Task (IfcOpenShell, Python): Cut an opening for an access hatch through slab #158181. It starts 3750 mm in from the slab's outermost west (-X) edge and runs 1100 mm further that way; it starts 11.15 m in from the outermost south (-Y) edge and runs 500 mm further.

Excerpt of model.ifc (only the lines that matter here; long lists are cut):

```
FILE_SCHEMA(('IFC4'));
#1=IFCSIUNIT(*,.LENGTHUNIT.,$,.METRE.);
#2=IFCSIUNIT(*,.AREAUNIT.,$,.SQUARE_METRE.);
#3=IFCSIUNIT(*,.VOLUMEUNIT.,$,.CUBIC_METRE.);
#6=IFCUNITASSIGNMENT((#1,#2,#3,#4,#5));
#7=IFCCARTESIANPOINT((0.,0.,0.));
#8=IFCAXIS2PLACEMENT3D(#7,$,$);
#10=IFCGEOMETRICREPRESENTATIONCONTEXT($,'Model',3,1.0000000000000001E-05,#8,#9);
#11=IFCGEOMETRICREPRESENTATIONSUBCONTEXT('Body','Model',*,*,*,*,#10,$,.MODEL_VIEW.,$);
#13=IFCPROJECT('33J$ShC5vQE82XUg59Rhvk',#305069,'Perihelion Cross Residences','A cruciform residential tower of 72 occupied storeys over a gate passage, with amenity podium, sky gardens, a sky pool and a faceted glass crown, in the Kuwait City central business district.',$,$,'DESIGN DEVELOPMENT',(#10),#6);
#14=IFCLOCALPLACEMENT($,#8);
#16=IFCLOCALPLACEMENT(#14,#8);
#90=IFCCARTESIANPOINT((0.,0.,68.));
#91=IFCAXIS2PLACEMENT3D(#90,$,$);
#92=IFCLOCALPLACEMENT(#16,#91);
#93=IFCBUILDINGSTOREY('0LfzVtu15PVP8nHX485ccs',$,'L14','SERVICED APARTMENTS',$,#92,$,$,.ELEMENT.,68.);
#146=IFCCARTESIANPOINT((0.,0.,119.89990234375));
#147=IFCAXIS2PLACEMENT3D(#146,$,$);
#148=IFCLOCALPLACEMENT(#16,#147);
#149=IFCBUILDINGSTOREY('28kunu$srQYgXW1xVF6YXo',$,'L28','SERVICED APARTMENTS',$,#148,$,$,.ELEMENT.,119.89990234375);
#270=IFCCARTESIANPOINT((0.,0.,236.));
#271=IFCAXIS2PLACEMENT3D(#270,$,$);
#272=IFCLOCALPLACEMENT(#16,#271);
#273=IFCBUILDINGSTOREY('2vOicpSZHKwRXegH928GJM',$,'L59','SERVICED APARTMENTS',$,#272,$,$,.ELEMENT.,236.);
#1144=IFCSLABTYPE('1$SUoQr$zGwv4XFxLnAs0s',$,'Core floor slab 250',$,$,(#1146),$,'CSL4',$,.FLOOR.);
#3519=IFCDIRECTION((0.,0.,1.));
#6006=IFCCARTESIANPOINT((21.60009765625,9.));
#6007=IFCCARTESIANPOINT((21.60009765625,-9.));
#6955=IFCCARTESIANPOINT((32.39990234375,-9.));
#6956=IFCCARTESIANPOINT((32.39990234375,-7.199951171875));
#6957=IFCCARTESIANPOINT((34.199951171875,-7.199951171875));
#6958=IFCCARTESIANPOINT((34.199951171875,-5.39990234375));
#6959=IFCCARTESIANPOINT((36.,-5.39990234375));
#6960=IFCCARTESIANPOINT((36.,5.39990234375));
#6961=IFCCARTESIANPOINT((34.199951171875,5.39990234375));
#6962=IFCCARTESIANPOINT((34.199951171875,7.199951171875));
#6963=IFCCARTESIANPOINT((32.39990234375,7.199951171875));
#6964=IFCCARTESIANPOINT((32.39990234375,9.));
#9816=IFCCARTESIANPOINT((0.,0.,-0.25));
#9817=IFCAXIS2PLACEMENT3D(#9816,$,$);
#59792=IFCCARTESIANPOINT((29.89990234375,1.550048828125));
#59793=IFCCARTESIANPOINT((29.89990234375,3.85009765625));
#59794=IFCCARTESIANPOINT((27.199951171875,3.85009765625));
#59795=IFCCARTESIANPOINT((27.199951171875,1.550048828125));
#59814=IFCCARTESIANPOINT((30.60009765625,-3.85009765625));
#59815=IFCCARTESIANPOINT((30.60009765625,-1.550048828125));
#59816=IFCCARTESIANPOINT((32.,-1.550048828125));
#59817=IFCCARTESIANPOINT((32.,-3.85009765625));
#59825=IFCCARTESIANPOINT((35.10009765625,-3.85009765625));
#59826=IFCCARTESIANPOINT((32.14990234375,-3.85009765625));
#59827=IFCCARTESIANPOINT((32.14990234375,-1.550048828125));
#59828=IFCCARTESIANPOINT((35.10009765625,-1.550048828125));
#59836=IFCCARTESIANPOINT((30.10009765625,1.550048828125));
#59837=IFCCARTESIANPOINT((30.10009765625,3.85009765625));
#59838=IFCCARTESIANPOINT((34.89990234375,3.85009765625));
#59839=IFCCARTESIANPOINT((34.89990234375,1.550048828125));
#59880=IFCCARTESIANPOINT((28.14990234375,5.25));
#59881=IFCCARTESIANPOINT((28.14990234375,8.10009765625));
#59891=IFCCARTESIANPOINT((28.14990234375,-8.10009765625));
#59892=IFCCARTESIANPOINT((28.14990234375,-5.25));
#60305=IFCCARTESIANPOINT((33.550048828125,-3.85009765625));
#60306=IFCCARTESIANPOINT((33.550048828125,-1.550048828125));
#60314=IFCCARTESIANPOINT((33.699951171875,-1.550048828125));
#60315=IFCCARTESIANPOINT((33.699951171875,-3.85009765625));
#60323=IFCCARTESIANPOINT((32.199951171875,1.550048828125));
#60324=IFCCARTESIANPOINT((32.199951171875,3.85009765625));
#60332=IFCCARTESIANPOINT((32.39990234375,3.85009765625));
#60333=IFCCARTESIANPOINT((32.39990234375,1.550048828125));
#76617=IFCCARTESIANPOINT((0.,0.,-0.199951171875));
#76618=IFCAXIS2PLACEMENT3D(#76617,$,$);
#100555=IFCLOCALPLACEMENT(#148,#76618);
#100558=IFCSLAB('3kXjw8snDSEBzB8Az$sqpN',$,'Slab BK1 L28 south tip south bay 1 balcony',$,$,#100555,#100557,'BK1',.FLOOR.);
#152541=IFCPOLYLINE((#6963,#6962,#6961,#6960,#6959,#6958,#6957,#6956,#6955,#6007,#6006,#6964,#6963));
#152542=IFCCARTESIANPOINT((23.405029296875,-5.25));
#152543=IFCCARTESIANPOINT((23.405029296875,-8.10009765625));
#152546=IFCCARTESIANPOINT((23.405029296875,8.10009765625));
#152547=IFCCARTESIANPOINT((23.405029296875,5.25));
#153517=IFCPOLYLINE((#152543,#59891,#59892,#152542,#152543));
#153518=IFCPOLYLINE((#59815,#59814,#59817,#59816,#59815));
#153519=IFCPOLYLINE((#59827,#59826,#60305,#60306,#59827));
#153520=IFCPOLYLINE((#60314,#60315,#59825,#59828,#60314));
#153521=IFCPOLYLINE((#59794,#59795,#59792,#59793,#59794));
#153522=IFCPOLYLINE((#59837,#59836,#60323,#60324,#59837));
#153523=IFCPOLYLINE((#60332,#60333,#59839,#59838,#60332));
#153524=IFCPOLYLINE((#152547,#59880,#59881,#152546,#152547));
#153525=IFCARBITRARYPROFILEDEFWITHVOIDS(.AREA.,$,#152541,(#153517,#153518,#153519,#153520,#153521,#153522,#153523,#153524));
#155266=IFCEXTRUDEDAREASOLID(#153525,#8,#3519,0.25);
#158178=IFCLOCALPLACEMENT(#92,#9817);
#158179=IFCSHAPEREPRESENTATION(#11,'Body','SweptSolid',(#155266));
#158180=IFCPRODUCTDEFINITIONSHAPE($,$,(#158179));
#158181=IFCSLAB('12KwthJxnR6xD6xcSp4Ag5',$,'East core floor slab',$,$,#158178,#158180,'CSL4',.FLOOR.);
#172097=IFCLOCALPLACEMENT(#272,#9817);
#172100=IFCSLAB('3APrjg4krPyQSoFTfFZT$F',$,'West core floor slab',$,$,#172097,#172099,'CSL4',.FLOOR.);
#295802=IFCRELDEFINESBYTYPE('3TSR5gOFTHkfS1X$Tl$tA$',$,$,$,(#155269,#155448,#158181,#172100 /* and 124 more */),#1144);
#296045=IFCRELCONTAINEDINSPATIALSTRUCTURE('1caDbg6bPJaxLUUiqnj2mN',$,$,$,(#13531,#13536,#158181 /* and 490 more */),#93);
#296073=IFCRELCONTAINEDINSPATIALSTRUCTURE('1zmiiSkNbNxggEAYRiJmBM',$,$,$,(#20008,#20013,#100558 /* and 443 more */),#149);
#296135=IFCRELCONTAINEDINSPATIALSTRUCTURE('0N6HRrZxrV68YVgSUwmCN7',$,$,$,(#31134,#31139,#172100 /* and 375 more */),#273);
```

```python
import numpy as np
import ifcopenshell
import ifcopenshell.api.feature
import ifcopenshell.api.geometry
import ifcopenshell.api.root
import ifcopenshell.geom
import ifcopenshell.util.placement
import ifcopenshell.util.representation
import ifcopenshell.util.shape
import ifcopenshell.util.unit

model = ifcopenshell.open("model.ifc")
unit_scale = ifcopenshell.util.unit.calculate_unit_scale(model)
settings = ifcopenshell.geom.settings()


def volume(element):
    """Net volume in cubic metres, openings subtracted."""
    shape = ifcopenshell.geom.create_shape(settings, element)
    return ifcopenshell.util.shape.get_volume(shape.geometry)


slab = model.by_id(158181)
before = volume(slab)

# Extent in the slab's own axes, in metres. The edges named are its -X and -Y sides.
slab_shape = ifcopenshell.geom.create_shape(settings, slab)
vertices = ifcopenshell.util.shape.get_vertices(slab_shape.geometry)
x_min, y_min, bottom = vertices.min(axis=0)
top = vertices[:, 2].max()

opening = ifcopenshell.api.root.create_entity(model, ifc_class="IfcOpeningElement", name="Access hatch opening", predefined_type="OPENING")
context = ifcopenshell.util.representation.get_context(model, "Model", "Body", "MODEL_VIEW")
width, depth = 1.1, 0.5
outline = [(0.0, 0.0), (width, 0.0), (width, depth), (0.0, depth), (0.0, 0.0)]
# Overshoot both faces by 50 mm so the cut is clean.
shape = ifcopenshell.api.geometry.add_slab_representation(
    model, context=context, depth=top - bottom + 0.1, polyline=outline
)
ifcopenshell.api.geometry.assign_representation(model, product=opening, representation=shape)

matrix = ifcopenshell.util.placement.get_local_placement(slab.ObjectPlacement)
matrix[:, 3] = matrix @ np.append(np.array([x_min + 3.75, y_min + 11.15, bottom - 0.05]) / unit_scale, 1.0)
ifcopenshell.api.geometry.edit_object_placement(model, product=opening, matrix=matrix, is_si=False)
ifcopenshell.api.feature.add_feature(model, feature=opening, element=slab)

after = volume(slab)

print(f"slab volume {before:.3f} -> {after:.3f} m3")

model.write("model_rev.ifc")
```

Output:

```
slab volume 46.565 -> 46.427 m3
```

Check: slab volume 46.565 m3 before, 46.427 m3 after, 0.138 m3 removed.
